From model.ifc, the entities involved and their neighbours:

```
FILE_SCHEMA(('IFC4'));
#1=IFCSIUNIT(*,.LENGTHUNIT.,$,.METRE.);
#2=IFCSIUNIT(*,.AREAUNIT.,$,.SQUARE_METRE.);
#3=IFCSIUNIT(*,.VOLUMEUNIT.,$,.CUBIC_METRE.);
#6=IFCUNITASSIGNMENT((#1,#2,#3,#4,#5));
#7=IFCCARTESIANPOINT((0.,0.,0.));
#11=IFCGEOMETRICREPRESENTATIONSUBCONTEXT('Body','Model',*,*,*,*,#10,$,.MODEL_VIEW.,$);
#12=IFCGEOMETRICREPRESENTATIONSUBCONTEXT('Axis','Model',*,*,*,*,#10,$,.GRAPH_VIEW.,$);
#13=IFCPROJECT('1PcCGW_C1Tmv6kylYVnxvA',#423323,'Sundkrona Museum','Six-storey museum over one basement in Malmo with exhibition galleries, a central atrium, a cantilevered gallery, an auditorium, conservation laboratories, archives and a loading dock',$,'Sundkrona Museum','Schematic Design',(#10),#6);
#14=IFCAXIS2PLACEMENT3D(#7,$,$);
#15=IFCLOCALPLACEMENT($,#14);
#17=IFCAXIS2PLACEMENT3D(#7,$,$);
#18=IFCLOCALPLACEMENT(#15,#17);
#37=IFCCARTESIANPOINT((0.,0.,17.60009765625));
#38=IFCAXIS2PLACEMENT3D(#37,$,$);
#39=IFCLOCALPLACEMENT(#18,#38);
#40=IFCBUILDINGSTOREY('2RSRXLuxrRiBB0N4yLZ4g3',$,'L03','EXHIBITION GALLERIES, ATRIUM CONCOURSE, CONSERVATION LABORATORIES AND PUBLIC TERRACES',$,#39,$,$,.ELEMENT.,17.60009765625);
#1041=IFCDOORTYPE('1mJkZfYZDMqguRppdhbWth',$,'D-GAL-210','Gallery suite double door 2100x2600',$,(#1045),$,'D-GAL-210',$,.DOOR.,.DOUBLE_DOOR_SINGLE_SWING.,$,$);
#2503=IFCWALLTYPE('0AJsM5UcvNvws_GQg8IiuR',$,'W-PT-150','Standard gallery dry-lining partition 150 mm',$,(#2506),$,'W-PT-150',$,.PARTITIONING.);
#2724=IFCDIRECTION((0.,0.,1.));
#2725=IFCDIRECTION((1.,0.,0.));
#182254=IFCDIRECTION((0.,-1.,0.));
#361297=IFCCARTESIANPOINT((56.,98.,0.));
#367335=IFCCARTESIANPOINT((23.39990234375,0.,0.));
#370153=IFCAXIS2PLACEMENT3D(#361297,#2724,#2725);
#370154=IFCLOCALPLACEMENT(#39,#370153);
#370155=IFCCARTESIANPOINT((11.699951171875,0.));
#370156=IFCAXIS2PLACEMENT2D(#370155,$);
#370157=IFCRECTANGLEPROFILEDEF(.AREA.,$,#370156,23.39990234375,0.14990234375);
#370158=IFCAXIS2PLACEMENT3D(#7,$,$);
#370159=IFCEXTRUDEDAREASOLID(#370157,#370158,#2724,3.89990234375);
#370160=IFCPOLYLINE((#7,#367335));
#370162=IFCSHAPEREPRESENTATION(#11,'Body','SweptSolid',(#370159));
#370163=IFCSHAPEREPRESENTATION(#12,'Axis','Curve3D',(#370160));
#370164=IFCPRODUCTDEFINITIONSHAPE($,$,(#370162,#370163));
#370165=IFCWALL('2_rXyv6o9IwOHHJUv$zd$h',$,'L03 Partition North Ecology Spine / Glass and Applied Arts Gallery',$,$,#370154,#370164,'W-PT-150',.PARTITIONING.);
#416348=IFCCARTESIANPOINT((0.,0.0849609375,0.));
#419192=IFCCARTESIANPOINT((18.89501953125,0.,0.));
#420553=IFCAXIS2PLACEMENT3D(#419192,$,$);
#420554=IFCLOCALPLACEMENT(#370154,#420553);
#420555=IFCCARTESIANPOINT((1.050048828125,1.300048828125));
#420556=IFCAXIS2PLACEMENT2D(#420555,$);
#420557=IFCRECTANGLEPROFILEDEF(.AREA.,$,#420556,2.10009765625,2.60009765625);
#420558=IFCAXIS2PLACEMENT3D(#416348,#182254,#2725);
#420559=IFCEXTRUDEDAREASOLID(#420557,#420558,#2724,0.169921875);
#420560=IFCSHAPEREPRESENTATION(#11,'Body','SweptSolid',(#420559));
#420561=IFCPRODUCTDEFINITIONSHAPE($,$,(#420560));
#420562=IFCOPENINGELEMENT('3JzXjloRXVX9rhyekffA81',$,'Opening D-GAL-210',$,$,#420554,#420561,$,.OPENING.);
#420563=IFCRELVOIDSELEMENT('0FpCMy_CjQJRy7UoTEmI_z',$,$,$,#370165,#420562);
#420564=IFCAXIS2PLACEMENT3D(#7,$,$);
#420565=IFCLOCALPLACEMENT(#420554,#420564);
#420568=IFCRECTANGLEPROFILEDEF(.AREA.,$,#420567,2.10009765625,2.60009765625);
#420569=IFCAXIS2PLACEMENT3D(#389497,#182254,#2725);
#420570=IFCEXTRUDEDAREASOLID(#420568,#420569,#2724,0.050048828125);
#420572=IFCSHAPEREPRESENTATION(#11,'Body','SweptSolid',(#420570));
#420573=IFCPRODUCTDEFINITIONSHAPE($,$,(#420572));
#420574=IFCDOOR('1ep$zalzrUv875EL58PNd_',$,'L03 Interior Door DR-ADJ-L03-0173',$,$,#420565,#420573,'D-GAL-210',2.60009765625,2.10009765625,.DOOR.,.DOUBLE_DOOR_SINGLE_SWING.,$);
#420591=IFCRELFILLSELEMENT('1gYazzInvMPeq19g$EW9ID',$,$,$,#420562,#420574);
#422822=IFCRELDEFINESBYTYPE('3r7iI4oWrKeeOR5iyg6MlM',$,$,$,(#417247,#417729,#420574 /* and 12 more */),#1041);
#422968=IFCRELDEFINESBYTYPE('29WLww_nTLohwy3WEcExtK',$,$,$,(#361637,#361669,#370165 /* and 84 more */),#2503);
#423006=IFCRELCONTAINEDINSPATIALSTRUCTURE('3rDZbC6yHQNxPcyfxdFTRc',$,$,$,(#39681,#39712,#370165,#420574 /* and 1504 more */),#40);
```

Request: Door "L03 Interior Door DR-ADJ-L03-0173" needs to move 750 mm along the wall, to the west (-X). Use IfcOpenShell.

```python
import ifcopenshell
import ifcopenshell.api.geometry
import ifcopenshell.util.placement
import ifcopenshell.util.unit

model = ifcopenshell.open("model.ifc")
unit_scale = ifcopenshell.util.unit.calculate_unit_scale(model)

door = model.by_guid("1ep$zalzrUv875EL58PNd_")
opening = door.FillsVoids[0].RelatingOpeningElement
wall = opening.VoidsElements[0].RelatingBuildingElement

wall_matrix = ifcopenshell.util.placement.get_local_placement(wall.ObjectPlacement)
shift = wall_matrix[:3, 0] * -0.75 / unit_scale
before = ifcopenshell.util.placement.get_local_placement(door.ObjectPlacement)[:3, 3].copy()

# The door is placed relative to its opening, so it follows when the opening moves.
matrix = ifcopenshell.util.placement.get_local_placement(opening.ObjectPlacement)
matrix[:3, 3] += shift
ifcopenshell.api.geometry.edit_object_placement(
    model, product=opening, matrix=matrix, is_si=False, should_transform_children=True
)

after = ifcopenshell.util.placement.get_local_placement(door.ObjectPlacement)[:3, 3]
print("door moved by", (after - before).round(3) + 0.0)

model.write("model_updated.ifc")
```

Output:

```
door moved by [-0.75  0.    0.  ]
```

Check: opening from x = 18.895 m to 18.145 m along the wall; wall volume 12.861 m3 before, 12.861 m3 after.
